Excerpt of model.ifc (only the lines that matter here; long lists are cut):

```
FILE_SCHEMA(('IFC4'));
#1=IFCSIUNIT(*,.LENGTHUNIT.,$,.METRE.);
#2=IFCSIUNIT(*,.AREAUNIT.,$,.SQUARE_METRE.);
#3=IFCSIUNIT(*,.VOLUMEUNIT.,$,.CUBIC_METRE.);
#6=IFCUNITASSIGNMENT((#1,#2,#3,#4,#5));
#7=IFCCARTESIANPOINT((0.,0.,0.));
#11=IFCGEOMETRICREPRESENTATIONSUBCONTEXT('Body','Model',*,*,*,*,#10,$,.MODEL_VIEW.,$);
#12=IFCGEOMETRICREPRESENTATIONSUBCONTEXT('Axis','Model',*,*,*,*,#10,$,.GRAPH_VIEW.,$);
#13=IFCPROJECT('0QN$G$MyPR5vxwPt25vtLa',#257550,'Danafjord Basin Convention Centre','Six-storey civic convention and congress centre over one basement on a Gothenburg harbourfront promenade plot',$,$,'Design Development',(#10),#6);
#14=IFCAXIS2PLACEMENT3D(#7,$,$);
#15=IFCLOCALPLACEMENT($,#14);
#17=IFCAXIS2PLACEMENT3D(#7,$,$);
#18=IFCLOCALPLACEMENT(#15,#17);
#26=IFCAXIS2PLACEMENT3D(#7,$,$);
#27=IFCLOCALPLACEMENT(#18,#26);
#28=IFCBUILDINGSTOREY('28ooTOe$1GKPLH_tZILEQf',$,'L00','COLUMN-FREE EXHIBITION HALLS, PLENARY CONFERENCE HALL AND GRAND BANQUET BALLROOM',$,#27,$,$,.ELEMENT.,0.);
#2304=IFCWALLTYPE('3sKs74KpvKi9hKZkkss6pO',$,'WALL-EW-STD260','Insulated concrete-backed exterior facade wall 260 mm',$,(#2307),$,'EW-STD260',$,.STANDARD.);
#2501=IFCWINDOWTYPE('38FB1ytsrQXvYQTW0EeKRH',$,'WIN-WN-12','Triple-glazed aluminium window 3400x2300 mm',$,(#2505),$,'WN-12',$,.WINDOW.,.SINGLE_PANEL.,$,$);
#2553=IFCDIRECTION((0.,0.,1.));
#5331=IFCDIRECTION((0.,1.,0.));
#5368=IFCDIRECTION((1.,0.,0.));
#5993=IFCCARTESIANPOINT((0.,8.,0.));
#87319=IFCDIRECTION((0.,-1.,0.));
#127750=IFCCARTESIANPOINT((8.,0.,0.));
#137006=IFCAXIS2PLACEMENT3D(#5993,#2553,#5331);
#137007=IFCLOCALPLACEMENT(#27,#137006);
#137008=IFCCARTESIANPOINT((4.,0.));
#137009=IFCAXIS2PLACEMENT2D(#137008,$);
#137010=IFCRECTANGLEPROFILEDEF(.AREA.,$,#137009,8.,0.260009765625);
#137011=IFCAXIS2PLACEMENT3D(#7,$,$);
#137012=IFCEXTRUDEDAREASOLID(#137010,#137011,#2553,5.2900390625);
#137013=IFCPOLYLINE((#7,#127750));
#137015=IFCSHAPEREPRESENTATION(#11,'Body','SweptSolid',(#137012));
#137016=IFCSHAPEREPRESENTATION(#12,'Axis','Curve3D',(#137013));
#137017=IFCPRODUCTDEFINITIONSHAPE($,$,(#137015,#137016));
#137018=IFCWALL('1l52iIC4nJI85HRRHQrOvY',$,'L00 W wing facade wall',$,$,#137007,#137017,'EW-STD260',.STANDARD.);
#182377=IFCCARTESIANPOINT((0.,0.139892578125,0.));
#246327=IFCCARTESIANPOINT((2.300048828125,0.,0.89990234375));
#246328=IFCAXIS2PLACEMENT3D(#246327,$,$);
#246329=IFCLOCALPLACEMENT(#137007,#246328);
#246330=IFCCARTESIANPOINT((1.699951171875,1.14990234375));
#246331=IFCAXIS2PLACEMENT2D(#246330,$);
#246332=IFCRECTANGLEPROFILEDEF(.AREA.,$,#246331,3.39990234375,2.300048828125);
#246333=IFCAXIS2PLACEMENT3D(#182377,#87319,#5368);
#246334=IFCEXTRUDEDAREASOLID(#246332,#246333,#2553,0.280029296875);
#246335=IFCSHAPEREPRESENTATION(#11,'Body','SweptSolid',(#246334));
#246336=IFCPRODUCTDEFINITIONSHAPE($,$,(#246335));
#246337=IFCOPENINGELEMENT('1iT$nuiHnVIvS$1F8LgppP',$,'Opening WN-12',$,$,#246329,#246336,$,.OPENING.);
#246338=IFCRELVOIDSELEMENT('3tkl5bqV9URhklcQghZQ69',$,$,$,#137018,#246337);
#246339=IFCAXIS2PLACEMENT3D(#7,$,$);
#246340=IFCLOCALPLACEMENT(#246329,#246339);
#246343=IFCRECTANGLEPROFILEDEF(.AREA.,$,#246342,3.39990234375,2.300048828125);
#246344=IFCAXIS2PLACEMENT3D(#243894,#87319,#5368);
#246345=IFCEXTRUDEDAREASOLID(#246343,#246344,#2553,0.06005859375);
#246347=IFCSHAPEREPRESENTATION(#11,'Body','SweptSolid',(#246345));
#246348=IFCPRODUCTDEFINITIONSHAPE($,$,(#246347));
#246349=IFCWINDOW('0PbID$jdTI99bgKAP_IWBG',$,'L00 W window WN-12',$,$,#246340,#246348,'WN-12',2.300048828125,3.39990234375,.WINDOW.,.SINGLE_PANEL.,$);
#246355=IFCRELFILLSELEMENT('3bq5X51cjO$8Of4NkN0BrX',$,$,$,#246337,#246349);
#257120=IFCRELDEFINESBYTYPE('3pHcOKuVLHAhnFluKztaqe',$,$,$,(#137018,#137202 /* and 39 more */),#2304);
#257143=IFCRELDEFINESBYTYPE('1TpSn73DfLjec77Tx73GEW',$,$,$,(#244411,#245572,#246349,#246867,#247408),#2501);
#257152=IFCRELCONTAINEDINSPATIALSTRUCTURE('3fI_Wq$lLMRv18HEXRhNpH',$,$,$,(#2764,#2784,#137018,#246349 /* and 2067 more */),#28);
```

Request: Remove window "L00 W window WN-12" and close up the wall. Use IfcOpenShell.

```python
import ifcopenshell
import ifcopenshell.api.feature
import ifcopenshell.api.root
import ifcopenshell.geom
import ifcopenshell.util.shape

model = ifcopenshell.open("model.ifc")
settings = ifcopenshell.geom.settings()


def volume(element):
    """Net volume in cubic metres, openings subtracted."""
    shape = ifcopenshell.geom.create_shape(settings, element)
    return ifcopenshell.util.shape.get_volume(shape.geometry)


window = model.by_id(246349)
opening = window.FillsVoids[0].RelatingOpeningElement
wall = opening.VoidsElements[0].RelatingBuildingElement
before = volume(wall)

ifcopenshell.api.root.remove_product(model, product=window)
ifcopenshell.api.feature.remove_feature(model, feature=opening)

after = volume(wall)

print(f"wall volume {before:.3f} -> {after:.3f} m3")

model.write("model_edited.ifc")
```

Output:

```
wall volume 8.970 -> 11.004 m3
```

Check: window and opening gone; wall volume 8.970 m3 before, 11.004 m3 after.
